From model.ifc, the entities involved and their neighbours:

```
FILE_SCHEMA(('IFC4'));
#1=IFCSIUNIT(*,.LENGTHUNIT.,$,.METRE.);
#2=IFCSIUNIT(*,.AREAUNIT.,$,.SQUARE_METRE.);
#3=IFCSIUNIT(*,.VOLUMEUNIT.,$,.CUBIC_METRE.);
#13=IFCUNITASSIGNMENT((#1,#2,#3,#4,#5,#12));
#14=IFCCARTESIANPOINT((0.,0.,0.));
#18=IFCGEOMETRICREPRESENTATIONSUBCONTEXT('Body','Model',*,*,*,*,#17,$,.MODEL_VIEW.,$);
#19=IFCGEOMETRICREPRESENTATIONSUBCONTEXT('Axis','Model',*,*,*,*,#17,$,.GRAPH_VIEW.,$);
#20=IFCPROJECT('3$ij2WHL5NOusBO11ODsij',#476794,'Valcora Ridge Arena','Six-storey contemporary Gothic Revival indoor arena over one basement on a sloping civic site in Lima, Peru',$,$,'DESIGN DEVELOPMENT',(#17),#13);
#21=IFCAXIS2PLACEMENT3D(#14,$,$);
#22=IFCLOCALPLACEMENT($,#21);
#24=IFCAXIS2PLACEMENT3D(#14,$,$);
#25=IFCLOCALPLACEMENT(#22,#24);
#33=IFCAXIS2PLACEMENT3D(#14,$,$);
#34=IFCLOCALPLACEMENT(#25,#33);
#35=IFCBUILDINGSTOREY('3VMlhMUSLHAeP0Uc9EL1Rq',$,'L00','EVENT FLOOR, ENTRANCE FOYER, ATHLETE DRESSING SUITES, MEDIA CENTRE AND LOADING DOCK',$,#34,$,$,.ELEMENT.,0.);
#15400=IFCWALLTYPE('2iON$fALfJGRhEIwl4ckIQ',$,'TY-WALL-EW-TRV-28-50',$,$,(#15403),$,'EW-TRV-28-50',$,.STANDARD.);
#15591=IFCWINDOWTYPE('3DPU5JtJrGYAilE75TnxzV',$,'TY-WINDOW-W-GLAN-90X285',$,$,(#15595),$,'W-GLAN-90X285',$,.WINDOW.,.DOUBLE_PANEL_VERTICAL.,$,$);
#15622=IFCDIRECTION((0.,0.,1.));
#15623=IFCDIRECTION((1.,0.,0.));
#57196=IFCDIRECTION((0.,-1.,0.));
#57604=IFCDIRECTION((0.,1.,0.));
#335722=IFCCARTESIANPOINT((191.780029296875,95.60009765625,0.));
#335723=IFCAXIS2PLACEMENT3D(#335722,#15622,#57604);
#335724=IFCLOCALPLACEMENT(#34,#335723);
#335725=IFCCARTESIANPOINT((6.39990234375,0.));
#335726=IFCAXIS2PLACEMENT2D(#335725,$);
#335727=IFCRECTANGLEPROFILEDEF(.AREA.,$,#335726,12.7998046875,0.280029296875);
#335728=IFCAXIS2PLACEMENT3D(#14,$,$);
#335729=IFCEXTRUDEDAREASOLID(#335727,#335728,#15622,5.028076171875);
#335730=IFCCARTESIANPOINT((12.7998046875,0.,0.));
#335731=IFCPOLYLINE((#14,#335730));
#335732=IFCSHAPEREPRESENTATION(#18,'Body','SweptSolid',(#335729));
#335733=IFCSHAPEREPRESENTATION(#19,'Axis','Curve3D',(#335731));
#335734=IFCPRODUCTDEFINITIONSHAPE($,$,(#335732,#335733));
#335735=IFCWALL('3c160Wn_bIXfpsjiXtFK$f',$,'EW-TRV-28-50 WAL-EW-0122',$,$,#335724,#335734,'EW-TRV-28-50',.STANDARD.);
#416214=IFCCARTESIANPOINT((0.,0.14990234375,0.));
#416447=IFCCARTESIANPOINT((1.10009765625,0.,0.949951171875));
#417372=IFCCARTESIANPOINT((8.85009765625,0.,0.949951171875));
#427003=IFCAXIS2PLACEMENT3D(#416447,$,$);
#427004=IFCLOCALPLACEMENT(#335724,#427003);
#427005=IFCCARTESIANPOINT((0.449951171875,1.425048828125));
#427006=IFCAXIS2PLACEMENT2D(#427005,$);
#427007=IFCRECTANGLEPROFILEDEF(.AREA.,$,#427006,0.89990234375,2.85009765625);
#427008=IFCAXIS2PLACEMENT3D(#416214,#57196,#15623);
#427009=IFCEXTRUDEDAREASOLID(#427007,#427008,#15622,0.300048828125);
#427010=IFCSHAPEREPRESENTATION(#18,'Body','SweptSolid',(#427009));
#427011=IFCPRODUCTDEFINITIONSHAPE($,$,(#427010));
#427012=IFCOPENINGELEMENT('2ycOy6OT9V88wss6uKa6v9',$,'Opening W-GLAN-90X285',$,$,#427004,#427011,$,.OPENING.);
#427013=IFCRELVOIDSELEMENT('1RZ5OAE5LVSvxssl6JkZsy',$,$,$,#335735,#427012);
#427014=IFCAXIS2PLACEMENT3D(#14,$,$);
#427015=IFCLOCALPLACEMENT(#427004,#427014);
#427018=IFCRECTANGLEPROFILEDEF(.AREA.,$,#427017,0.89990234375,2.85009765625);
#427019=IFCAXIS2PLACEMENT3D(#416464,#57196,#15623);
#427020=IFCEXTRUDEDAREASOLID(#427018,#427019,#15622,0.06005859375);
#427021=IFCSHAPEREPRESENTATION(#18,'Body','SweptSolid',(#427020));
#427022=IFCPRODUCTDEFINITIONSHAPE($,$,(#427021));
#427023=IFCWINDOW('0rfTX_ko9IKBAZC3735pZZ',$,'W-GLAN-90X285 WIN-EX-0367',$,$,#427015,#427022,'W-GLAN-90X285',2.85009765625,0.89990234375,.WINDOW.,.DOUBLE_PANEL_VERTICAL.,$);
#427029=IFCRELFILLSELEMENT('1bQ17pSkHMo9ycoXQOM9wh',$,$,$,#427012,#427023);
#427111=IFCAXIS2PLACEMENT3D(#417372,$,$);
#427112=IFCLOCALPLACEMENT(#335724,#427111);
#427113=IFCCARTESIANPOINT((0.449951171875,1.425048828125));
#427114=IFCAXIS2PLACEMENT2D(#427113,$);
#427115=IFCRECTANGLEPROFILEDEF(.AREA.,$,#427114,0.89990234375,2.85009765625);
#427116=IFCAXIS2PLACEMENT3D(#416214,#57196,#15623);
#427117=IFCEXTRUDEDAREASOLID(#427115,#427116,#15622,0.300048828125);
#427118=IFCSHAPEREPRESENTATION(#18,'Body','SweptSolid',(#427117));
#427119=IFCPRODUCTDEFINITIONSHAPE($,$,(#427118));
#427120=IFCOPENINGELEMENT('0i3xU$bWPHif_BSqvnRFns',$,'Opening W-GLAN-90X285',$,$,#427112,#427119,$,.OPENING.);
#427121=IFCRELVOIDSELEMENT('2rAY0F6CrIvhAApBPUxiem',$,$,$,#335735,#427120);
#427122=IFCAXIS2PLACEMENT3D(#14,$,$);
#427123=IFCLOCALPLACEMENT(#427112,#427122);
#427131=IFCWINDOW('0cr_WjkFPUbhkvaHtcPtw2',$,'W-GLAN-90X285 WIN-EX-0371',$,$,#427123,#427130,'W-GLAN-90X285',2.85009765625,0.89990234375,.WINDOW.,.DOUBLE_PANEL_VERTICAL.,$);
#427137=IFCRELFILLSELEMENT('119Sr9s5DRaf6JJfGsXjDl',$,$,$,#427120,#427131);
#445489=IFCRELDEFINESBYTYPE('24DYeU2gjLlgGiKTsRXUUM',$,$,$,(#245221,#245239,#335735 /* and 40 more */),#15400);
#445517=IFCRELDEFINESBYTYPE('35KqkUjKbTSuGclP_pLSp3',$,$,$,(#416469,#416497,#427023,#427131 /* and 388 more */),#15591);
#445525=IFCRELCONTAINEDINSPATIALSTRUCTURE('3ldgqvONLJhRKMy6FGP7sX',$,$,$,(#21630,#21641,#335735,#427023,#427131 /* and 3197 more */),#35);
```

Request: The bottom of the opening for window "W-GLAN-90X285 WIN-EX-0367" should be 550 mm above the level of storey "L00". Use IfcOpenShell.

```python
import numpy as np
import ifcopenshell
import ifcopenshell.api.geometry
import ifcopenshell.geom
import ifcopenshell.util.element
import ifcopenshell.util.placement
import ifcopenshell.util.shape
import ifcopenshell.util.unit

model = ifcopenshell.open("model.ifc")
unit_scale = ifcopenshell.util.unit.calculate_unit_scale(model)

window = model.by_guid("0rfTX_ko9IKBAZC3735pZZ")
opening = window.FillsVoids[0].RelatingOpeningElement
storey = ifcopenshell.util.element.get_container(window, ifc_class="IfcBuildingStorey")
level = ifcopenshell.util.placement.get_local_placement(storey.ObjectPlacement)[2, 3]

# The opening's origin need not be at the sill, so measure its lowest point.
shape = ifcopenshell.geom.create_shape(ifcopenshell.geom.settings(), opening)
bottom = ifcopenshell.util.shape.get_shape_bottom_elevation(shape, shape.geometry) / unit_scale
dz = level + 0.55 / unit_scale - bottom

shift = np.array([0.0, 0.0, dz])
# The window is placed relative to its opening, so it follows when the opening moves.
matrix = ifcopenshell.util.placement.get_local_placement(opening.ObjectPlacement)
matrix[:3, 3] += shift
ifcopenshell.api.geometry.edit_object_placement(
    model, product=opening, matrix=matrix, is_si=False, should_transform_children=True
)

print(f"moved by {dz * unit_scale:+.3f} m")

model.write("model_updated.ifc")
```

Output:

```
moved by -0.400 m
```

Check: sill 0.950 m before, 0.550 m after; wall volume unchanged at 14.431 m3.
